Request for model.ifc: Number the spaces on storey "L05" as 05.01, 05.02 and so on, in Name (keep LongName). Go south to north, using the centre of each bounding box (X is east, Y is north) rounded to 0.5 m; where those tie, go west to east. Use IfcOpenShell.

First a look at what the model holds.

```python
import ifcopenshell
import ifcopenshell.util.element
import ifcopenshell.util.placement

model = ifcopenshell.open("model.ifc")
print(model.schema)
storey = next(s for s in model.by_type("IfcBuildingStorey") if s.Name == "L05")
spaces = [e for e in ifcopenshell.util.element.get_decomposition(storey) if e.is_a("IfcSpace")]
for e in sorted(spaces, key=lambda e: e.id()):
    origin = ifcopenshell.util.placement.get_local_placement(e.ObjectPlacement)[:3, 3]
    print(e.id(), e.Name, e.LongName, origin.round(2) + 0.0, sep=" | ")
```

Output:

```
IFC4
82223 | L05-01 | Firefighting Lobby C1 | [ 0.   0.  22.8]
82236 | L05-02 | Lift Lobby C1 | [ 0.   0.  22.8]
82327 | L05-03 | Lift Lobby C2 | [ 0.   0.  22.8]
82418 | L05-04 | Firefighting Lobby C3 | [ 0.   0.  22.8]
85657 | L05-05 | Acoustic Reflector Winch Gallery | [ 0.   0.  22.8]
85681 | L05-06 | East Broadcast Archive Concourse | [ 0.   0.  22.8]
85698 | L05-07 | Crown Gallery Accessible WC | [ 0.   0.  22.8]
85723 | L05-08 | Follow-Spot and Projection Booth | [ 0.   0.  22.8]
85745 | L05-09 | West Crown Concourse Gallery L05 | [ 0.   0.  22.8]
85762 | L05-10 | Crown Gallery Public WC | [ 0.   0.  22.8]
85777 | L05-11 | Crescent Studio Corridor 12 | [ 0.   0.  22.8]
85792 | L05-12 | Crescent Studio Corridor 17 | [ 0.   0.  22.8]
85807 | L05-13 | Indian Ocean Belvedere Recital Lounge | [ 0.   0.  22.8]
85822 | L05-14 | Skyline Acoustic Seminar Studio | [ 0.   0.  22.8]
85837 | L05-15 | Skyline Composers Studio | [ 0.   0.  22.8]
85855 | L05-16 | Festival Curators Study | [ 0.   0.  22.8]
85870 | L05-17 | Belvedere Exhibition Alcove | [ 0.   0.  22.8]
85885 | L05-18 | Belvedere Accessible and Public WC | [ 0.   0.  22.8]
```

```python
import ifcopenshell
import ifcopenshell.geom
import ifcopenshell.util.element
import ifcopenshell.util.shape

model = ifcopenshell.open("model.ifc")
settings = ifcopenshell.geom.settings()
settings.set("use-world-coords", True)


def centre(element):
    shape = ifcopenshell.geom.create_shape(settings, element)
    return ifcopenshell.util.shape.get_bbox_centroid(shape.geometry)


storey = next(s for s in model.by_type("IfcBuildingStorey") if s.Name == "L05")
spaces = [e for e in ifcopenshell.util.element.get_decomposition(storey) if e.is_a("IfcSpace")]

# Insertion points can sit at a corner or the storey origin, so sort by the geometry (in metres).
centres = {e: centre(e) for e in spaces}
spaces.sort(key=lambda e: (round(centres[e][1] / 0.5), centres[e][0]))

for i, e in enumerate(spaces, start=1):
    number = f"05.{i:02d}"
    e.Name = number
    print(e.id(), number)

model.write("model_rev.ifc")
```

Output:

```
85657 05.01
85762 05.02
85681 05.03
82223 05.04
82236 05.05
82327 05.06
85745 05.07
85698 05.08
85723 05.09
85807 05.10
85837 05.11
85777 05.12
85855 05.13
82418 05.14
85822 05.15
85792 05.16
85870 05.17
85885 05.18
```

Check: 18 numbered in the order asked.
